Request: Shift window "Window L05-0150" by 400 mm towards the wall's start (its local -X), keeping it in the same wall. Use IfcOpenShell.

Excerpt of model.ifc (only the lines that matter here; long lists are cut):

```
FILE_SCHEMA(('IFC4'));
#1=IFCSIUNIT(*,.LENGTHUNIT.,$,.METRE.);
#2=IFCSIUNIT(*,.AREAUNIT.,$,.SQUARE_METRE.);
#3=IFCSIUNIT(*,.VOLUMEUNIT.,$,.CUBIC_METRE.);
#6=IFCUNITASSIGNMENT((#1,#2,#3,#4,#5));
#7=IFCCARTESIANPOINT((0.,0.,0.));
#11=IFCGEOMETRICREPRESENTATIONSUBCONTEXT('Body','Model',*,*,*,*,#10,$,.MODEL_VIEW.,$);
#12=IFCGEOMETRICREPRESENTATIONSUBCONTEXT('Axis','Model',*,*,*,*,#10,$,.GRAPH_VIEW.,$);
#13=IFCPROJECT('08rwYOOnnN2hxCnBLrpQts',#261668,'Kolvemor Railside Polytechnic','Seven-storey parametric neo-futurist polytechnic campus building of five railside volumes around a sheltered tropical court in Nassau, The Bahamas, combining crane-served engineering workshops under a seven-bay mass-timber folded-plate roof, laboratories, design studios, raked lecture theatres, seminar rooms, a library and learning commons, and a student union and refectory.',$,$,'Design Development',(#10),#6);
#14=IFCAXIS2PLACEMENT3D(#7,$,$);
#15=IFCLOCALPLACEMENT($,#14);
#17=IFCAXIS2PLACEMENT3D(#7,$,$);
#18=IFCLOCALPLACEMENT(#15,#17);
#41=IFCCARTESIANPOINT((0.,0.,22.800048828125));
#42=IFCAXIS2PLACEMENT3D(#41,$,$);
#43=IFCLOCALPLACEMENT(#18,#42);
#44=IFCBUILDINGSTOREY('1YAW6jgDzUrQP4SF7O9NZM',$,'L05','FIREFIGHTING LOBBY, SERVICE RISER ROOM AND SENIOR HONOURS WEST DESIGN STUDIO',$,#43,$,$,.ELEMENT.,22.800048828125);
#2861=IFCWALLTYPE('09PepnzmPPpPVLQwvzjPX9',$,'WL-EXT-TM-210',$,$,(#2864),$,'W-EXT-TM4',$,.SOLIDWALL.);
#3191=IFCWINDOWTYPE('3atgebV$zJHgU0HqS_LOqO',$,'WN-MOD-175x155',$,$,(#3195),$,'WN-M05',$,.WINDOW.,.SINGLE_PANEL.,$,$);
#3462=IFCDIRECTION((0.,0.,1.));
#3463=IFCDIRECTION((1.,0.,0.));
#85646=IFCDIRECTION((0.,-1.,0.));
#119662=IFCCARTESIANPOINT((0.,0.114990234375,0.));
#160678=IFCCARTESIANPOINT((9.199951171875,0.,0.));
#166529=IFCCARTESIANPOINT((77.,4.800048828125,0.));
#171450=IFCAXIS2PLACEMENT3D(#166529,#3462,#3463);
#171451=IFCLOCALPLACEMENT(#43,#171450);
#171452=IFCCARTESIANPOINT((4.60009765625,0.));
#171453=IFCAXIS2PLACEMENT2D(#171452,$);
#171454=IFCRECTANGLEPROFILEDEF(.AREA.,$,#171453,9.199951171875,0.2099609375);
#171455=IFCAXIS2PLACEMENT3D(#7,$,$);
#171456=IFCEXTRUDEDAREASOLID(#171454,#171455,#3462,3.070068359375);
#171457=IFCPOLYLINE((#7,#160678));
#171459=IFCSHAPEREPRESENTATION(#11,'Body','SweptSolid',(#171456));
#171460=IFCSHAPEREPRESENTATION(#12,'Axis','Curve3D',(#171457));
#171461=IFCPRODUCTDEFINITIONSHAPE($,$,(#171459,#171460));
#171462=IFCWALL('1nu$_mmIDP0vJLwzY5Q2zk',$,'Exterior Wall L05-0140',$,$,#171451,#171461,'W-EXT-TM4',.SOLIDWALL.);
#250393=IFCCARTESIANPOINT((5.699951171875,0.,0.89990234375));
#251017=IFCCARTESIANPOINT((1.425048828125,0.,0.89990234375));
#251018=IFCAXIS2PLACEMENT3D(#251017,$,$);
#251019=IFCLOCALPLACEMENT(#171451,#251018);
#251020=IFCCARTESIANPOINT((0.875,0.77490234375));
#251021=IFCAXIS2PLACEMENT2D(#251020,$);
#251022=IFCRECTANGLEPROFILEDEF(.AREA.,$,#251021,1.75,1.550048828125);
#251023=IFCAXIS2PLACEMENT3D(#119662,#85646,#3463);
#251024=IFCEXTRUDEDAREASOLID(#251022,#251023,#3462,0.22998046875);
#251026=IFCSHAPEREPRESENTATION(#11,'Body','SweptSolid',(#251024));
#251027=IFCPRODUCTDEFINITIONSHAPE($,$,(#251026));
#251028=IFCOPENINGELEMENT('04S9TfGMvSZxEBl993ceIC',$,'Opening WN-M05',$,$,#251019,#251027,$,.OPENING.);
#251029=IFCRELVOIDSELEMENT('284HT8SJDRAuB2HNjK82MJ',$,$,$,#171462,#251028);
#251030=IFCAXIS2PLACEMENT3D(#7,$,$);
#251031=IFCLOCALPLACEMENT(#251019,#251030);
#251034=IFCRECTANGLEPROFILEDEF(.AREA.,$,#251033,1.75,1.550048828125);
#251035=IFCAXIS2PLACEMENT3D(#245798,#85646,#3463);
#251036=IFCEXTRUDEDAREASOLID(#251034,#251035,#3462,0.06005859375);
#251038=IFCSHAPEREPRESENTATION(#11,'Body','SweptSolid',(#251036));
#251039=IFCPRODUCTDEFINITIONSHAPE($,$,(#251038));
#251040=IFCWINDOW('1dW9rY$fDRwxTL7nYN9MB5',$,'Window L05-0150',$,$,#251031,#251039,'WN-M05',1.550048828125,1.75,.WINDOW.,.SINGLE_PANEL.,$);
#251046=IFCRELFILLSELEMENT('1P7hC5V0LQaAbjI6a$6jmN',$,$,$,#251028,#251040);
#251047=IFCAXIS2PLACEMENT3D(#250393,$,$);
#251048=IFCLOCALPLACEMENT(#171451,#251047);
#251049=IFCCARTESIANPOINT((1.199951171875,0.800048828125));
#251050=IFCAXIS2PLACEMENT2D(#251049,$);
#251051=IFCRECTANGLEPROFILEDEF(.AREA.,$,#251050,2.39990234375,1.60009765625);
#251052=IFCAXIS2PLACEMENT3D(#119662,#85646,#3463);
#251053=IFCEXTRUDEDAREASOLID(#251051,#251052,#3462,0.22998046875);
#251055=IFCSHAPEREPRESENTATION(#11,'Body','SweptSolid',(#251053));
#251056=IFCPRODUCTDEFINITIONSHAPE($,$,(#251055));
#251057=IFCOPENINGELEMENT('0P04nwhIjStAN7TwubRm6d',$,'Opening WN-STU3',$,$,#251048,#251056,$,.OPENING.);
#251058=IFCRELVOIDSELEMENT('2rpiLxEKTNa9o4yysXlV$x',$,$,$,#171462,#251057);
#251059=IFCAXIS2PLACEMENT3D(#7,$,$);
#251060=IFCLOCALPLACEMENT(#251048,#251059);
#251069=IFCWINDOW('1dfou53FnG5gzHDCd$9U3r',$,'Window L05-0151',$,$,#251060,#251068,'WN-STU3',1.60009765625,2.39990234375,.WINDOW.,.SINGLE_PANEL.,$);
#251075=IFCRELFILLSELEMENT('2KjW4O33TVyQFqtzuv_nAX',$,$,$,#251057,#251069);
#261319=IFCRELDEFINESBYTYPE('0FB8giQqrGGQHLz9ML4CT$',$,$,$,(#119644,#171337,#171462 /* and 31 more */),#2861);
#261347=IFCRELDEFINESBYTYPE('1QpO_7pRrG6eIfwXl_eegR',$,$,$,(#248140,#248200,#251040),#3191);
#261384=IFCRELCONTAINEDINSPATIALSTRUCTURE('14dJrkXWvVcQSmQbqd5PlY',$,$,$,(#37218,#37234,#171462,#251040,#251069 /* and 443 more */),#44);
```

```python
import ifcopenshell
import ifcopenshell.api.geometry
import ifcopenshell.util.placement
import ifcopenshell.util.unit

model = ifcopenshell.open("model.ifc")
unit_scale = ifcopenshell.util.unit.calculate_unit_scale(model)

window = model.by_guid("1dW9rY$fDRwxTL7nYN9MB5")
opening = window.FillsVoids[0].RelatingOpeningElement
wall = opening.VoidsElements[0].RelatingBuildingElement

wall_matrix = ifcopenshell.util.placement.get_local_placement(wall.ObjectPlacement)
shift = wall_matrix[:3, 0] * -0.4 / unit_scale
before = ifcopenshell.util.placement.get_local_placement(window.ObjectPlacement)[:3, 3].copy()

# The window is placed relative to its opening, so it follows when the opening moves.
matrix = ifcopenshell.util.placement.get_local_placement(opening.ObjectPlacement)
matrix[:3, 3] += shift
ifcopenshell.api.geometry.edit_object_placement(
    model, product=opening, matrix=matrix, is_si=False, should_transform_children=True
)

after = ifcopenshell.util.placement.get_local_placement(window.ObjectPlacement)[:3, 3]
print("window moved by", (after - before).round(3) + 0.0)

model.write("model-out.ifc")
```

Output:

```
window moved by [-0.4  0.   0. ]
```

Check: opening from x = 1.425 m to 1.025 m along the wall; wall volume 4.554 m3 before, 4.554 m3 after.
